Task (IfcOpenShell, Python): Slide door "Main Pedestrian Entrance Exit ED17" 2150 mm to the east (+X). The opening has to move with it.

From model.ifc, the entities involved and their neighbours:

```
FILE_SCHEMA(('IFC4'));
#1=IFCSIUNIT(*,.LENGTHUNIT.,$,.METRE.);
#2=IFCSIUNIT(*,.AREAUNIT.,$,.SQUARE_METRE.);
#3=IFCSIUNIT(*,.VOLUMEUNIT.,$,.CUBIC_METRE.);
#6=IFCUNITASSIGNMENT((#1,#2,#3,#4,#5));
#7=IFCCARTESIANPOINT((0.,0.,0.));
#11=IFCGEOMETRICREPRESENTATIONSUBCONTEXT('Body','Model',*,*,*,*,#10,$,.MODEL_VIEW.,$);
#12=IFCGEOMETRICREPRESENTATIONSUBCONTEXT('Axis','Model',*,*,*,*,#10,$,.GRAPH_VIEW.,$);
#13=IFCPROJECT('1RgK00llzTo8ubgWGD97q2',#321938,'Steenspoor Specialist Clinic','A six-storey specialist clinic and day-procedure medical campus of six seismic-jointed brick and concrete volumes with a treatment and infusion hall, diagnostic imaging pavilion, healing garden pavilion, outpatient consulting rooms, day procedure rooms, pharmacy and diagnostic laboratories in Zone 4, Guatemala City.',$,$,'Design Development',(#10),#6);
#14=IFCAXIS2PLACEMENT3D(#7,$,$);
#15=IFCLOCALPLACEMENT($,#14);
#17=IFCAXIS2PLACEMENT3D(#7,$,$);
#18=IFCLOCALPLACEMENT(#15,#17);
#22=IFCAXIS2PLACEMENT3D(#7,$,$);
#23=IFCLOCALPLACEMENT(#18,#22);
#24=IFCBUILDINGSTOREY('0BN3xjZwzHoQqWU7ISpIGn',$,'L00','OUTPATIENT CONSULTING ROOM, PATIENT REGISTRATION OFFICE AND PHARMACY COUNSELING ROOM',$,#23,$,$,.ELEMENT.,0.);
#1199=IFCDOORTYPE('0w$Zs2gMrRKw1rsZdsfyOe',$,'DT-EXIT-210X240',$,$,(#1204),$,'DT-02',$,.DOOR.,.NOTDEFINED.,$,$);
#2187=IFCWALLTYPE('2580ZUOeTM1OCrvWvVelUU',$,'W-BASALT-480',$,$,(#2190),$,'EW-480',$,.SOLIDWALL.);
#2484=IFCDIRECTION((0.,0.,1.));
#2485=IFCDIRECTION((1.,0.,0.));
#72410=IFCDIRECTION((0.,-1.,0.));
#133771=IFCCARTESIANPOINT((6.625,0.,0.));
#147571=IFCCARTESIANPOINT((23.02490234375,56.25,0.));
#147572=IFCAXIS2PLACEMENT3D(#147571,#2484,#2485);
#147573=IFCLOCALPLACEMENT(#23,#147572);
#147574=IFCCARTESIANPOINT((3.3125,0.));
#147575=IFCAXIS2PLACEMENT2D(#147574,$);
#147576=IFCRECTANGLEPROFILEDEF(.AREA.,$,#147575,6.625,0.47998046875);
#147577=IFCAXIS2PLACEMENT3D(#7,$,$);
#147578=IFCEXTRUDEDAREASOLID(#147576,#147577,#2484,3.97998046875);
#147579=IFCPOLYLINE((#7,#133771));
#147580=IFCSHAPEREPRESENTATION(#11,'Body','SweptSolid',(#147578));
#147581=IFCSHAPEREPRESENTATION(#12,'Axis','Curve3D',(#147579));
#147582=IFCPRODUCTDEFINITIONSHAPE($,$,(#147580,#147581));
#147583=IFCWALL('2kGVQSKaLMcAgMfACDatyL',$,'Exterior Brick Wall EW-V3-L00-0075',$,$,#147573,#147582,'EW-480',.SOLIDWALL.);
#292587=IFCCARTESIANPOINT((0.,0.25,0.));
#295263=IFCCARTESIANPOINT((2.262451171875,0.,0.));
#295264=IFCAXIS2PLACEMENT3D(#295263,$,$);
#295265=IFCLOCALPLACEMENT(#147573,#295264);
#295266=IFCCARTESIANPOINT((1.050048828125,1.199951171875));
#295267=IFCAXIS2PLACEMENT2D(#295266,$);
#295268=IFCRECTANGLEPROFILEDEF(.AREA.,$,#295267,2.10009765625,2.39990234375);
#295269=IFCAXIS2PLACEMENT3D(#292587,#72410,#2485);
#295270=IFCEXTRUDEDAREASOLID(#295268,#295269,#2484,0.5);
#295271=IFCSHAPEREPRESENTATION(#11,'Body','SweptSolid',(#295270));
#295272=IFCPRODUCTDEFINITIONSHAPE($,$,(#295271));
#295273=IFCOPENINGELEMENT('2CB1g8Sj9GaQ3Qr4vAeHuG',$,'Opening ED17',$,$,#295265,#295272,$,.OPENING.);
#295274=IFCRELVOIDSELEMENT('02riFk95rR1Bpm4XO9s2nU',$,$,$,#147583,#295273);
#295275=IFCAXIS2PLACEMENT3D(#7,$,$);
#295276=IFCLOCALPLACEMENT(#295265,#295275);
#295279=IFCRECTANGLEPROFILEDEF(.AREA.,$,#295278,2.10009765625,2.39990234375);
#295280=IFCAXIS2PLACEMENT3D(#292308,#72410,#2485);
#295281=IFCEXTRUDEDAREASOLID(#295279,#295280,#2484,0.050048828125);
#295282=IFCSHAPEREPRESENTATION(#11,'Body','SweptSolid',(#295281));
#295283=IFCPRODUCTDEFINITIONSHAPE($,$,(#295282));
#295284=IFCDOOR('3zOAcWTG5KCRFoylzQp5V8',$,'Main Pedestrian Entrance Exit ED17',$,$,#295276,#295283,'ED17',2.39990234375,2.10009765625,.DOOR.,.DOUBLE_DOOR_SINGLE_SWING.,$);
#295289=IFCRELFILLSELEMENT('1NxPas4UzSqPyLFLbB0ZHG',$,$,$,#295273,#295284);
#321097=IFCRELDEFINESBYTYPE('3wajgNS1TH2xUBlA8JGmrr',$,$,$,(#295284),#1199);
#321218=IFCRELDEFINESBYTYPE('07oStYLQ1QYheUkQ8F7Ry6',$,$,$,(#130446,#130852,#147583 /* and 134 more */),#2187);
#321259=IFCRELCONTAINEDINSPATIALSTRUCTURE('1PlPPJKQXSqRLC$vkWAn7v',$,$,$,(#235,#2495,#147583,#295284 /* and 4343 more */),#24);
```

```python
import ifcopenshell
import ifcopenshell.api.geometry
import ifcopenshell.util.placement

model = ifcopenshell.open("model.ifc")

door = model.by_guid("3zOAcWTG5KCRFoylzQp5V8")
opening = door.FillsVoids[0].RelatingOpeningElement
wall = opening.VoidsElements[0].RelatingBuildingElement

wall_matrix = ifcopenshell.util.placement.get_local_placement(wall.ObjectPlacement)
shift = wall_matrix[:3, 0] * 2.15
before = ifcopenshell.util.placement.get_local_placement(door.ObjectPlacement)[:3, 3].copy()

# The door is placed relative to its opening, so it follows when the opening moves.
matrix = ifcopenshell.util.placement.get_local_placement(opening.ObjectPlacement)
matrix[:3, 3] += shift
ifcopenshell.api.geometry.edit_object_placement(
    model, product=opening, matrix=matrix, is_si=False, should_transform_children=True
)

after = ifcopenshell.util.placement.get_local_placement(door.ObjectPlacement)[:3, 3]
print("door moved by", (after - before).round(3) + 0.0)

model.write("model_rev.ifc")
```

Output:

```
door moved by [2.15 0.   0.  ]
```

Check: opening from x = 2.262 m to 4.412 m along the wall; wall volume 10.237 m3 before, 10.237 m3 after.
